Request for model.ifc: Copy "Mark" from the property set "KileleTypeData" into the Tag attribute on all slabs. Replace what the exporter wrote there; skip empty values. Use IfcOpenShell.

First a look at what the model holds.

```python
import ifcopenshell
import ifcopenshell.util.element

model = ifcopenshell.open("model.ifc")
print(model.schema)
slabs = model.by_type("IfcSlab")
print(len(slabs), "slabs")
for e in slabs[:8]:
    source = ifcopenshell.util.element.get_pset(e, "KileleTypeData", "Mark")
    target = e.Tag
    print(e.id(), repr(source), repr(target), sep=" | ")
```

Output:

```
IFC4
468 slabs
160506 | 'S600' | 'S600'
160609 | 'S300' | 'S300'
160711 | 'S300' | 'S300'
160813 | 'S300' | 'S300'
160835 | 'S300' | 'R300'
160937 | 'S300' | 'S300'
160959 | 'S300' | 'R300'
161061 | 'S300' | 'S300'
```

```python
import ifcopenshell
import ifcopenshell.util.element

model = ifcopenshell.open("model.ifc")

count = 0
for e in model.by_type("IfcSlab"):
    value = ifcopenshell.util.element.get_pset(e, "KileleTypeData", "Mark")
    current = e.Tag
    if not value or not value.strip() or current == value:
        continue
    e.Tag = value
    count += 1

print(count, "slabs updated")

model.write("model_edited.ifc")
```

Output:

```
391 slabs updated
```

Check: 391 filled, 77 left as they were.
